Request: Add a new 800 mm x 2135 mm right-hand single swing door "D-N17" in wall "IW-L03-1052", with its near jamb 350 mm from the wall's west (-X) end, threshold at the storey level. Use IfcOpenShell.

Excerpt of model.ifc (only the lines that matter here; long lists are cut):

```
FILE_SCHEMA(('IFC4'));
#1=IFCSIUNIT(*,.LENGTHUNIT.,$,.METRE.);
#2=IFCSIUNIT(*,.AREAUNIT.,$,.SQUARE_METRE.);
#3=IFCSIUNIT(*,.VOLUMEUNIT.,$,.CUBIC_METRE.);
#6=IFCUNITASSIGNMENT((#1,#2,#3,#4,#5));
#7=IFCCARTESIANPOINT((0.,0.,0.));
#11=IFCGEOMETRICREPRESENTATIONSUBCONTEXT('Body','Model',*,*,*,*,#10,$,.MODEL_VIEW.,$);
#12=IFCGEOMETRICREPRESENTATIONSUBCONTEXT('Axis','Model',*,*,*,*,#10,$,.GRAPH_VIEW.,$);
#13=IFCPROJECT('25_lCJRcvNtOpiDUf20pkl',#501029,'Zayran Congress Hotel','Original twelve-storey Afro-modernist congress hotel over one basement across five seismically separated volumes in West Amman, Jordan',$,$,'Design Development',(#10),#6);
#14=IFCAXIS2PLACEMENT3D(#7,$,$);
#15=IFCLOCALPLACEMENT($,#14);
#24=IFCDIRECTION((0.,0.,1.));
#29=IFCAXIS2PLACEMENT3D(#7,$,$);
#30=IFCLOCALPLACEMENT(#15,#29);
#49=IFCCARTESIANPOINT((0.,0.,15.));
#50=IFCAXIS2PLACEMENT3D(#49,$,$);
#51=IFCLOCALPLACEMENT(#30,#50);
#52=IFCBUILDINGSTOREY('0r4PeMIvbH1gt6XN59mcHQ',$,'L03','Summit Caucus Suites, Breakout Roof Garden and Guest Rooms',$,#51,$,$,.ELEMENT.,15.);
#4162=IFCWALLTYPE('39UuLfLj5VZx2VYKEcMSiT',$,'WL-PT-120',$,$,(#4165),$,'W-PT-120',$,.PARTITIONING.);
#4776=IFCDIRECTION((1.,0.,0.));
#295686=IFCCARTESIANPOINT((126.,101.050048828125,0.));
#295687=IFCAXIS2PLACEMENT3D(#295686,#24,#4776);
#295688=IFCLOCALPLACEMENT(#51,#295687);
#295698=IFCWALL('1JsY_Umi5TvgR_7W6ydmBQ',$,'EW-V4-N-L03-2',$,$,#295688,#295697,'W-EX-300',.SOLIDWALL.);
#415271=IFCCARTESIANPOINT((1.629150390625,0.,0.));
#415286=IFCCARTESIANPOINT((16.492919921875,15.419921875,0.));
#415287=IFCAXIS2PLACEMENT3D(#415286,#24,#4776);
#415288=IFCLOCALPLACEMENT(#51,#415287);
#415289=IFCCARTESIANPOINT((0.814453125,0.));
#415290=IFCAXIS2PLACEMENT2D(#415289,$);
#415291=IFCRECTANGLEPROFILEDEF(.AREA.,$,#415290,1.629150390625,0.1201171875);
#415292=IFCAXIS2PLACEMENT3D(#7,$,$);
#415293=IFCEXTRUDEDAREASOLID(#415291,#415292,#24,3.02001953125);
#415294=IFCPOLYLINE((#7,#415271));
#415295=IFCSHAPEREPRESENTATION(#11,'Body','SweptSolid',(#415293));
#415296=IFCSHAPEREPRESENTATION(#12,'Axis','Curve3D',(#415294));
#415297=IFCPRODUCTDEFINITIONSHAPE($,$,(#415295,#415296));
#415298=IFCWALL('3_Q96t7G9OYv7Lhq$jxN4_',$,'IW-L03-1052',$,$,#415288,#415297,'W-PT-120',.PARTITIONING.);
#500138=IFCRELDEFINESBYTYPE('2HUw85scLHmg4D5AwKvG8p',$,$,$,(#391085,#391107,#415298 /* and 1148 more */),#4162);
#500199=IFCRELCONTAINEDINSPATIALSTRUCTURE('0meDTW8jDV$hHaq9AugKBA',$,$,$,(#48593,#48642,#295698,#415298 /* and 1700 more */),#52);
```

```python
import numpy as np
import ifcopenshell
import ifcopenshell.api.feature
import ifcopenshell.api.geometry
import ifcopenshell.api.root
import ifcopenshell.api.spatial
import ifcopenshell.geom
import ifcopenshell.util.element
import ifcopenshell.util.placement
import ifcopenshell.util.representation
import ifcopenshell.util.shape
import ifcopenshell.util.unit

model = ifcopenshell.open("model.ifc")
unit_scale = ifcopenshell.util.unit.calculate_unit_scale(model)
settings = ifcopenshell.geom.settings()


def volume(element):
    """Net volume in cubic metres, openings subtracted."""
    shape = ifcopenshell.geom.create_shape(settings, element)
    return ifcopenshell.util.shape.get_volume(shape.geometry)


wall = model.by_id(415298)
storey = ifcopenshell.util.element.get_container(wall, ifc_class="IfcBuildingStorey")
context = ifcopenshell.util.representation.get_context(model, "Model", "Body", "MODEL_VIEW")
before = volume(wall)

width, height, from_end, sill = 0.8, 2.135, 0.35, 0.0  # metres

# The wall runs along its own X axis, and the end named is its -X end.
wall_shape = ifcopenshell.geom.create_shape(settings, wall)
x, y, z = ifcopenshell.util.shape.get_vertices(wall_shape.geometry).T
start = x.min() + from_end
face, thickness = float(y.min()), float(y.max() - y.min())
wall_matrix = ifcopenshell.util.placement.get_local_placement(wall.ObjectPlacement)
level = ifcopenshell.util.placement.get_local_placement(storey.ObjectPlacement)[2, 3]


def in_wall(x, y):
    """Placement at x, y metres in the wall's axes, at sill height."""
    matrix = wall_matrix.copy()
    matrix[:, 3] = wall_matrix @ np.array([x / unit_scale, y / unit_scale, 0.0, 1.0])
    matrix[2, 3] = level + sill / unit_scale
    return matrix


# Opening: a box that overshoots both wall faces by 50 mm.
opening = ifcopenshell.api.root.create_entity(model, ifc_class="IfcOpeningElement", predefined_type="OPENING")
box = ifcopenshell.api.geometry.add_wall_representation(
    model, context=context, length=width, height=height, thickness=thickness + 0.1
)
ifcopenshell.api.geometry.assign_representation(model, product=opening, representation=box)
ifcopenshell.api.geometry.edit_object_placement(model, product=opening, matrix=in_wall(start, face - 0.05), is_si=False)
ifcopenshell.api.feature.add_feature(model, feature=opening, element=wall)

door = ifcopenshell.api.root.create_entity(model, ifc_class="IfcDoor", name="D-N17", predefined_type="DOOR")
door.OverallWidth, door.OverallHeight = width / unit_scale, height / unit_scale
door.OperationType = "SINGLE_SWING_RIGHT"
body = ifcopenshell.api.geometry.add_door_representation(
    model,
    context=context,
    overall_width=door.OverallWidth,
    overall_height=door.OverallHeight,
    operation_type="SINGLE_SWING_RIGHT",
    lining_properties={"LiningDepth": thickness / unit_scale, "ThresholdDepth": thickness / unit_scale},
)
ifcopenshell.api.geometry.assign_representation(model, product=door, representation=body)
ifcopenshell.api.spatial.assign_container(model, products=[door], relating_structure=storey)
ifcopenshell.api.feature.add_filling(model, opening=opening, element=door)

# The lining spans the wall, so the door starts at the wall face.
ifcopenshell.api.geometry.edit_object_placement(model, product=door, matrix=in_wall(start, face), is_si=False)

after = volume(wall)

print(f"wall volume {before:.3f} -> {after:.3f} m3")

model.write("model_edited.ifc")
```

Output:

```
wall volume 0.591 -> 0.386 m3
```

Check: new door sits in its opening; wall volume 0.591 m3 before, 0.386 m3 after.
